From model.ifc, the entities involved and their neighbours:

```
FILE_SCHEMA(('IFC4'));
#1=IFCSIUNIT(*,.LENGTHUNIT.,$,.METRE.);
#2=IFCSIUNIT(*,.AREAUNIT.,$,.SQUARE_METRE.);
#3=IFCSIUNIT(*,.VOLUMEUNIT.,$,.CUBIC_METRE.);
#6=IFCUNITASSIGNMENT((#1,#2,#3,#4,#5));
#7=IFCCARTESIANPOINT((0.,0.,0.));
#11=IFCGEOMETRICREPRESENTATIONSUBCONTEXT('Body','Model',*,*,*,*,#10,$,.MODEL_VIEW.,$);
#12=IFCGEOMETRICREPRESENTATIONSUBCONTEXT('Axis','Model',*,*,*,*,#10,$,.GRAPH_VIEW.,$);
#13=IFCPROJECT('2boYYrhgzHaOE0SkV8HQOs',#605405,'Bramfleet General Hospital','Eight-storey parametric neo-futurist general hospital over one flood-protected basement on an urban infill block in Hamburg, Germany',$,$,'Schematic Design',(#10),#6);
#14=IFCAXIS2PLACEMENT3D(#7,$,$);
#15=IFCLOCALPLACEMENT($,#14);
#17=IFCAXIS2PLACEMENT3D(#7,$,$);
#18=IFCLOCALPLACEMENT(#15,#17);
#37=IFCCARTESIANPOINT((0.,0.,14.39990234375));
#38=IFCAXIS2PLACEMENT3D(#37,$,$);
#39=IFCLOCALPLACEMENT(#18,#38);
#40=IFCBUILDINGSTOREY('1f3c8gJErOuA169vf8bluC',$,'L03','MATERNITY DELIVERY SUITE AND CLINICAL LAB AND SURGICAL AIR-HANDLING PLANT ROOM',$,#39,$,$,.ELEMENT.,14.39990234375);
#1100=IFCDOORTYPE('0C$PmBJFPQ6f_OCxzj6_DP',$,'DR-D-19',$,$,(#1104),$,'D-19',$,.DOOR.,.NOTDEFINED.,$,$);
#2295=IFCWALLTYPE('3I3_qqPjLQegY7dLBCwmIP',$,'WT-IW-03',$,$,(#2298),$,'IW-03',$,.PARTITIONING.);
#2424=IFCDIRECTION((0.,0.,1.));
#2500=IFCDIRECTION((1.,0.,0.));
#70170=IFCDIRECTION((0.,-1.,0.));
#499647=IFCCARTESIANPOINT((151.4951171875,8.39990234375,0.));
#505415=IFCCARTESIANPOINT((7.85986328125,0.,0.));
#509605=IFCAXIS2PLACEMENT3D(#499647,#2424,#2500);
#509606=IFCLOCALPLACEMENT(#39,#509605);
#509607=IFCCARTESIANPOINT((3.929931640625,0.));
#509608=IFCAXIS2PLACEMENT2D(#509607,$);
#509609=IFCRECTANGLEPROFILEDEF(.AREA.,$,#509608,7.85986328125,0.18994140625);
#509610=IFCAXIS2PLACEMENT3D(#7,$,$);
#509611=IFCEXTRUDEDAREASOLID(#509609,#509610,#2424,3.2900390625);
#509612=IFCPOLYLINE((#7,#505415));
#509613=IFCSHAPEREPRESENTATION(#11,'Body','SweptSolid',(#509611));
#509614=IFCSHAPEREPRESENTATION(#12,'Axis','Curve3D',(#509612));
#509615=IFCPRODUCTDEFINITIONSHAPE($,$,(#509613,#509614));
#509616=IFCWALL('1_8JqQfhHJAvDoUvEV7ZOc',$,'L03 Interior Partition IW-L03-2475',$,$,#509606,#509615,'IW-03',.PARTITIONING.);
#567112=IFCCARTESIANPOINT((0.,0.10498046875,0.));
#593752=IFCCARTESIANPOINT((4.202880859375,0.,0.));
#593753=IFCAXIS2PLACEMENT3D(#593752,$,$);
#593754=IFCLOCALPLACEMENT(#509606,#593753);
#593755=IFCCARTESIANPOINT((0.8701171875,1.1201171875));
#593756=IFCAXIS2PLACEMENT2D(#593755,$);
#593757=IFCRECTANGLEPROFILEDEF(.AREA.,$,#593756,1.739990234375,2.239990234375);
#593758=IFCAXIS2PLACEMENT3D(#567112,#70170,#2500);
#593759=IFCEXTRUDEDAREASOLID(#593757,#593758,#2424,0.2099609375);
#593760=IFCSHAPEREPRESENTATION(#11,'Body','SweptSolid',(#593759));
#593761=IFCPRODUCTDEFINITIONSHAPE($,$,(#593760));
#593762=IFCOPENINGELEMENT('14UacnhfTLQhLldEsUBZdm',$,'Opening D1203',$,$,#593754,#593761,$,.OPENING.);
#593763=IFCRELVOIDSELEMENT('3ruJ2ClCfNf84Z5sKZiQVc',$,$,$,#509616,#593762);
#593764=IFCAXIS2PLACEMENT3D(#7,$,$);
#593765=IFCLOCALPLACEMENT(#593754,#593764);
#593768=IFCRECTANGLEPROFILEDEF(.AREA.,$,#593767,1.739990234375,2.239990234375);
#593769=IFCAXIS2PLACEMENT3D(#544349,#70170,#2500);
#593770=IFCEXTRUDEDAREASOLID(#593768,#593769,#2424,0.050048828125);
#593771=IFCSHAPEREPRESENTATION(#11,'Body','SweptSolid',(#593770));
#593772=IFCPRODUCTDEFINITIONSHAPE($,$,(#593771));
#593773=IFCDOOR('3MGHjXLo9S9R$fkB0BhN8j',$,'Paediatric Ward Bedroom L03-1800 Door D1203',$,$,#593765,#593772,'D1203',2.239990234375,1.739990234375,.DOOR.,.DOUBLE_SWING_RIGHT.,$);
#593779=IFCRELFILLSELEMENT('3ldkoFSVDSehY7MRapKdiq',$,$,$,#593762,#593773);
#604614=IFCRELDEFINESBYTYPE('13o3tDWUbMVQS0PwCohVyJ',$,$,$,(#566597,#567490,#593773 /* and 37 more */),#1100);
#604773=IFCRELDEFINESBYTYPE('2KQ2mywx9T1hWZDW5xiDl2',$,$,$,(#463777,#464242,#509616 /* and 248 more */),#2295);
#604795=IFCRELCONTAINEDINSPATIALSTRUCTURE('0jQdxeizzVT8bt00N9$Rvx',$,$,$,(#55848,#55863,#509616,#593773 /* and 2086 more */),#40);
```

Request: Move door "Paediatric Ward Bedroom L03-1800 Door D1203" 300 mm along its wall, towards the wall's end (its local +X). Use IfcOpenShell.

```python
import ifcopenshell
import ifcopenshell.api.geometry
import ifcopenshell.util.placement

model = ifcopenshell.open("model.ifc")

door = model.by_guid("3MGHjXLo9S9R$fkB0BhN8j")
opening = door.FillsVoids[0].RelatingOpeningElement
wall = opening.VoidsElements[0].RelatingBuildingElement

wall_matrix = ifcopenshell.util.placement.get_local_placement(wall.ObjectPlacement)
shift = wall_matrix[:3, 0] * 0.3
before = ifcopenshell.util.placement.get_local_placement(door.ObjectPlacement)[:3, 3].copy()

# The door is placed relative to its opening, so it follows when the opening moves.
matrix = ifcopenshell.util.placement.get_local_placement(opening.ObjectPlacement)
matrix[:3, 3] += shift
ifcopenshell.api.geometry.edit_object_placement(
    model, product=opening, matrix=matrix, is_si=False, should_transform_children=True
)

after = ifcopenshell.util.placement.get_local_placement(door.ObjectPlacement)[:3, 3]
print("door moved by", (after - before).round(3) + 0.0)

model.write("model_updated.ifc")
```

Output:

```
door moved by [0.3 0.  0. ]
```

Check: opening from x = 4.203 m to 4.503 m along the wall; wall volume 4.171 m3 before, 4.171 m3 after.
